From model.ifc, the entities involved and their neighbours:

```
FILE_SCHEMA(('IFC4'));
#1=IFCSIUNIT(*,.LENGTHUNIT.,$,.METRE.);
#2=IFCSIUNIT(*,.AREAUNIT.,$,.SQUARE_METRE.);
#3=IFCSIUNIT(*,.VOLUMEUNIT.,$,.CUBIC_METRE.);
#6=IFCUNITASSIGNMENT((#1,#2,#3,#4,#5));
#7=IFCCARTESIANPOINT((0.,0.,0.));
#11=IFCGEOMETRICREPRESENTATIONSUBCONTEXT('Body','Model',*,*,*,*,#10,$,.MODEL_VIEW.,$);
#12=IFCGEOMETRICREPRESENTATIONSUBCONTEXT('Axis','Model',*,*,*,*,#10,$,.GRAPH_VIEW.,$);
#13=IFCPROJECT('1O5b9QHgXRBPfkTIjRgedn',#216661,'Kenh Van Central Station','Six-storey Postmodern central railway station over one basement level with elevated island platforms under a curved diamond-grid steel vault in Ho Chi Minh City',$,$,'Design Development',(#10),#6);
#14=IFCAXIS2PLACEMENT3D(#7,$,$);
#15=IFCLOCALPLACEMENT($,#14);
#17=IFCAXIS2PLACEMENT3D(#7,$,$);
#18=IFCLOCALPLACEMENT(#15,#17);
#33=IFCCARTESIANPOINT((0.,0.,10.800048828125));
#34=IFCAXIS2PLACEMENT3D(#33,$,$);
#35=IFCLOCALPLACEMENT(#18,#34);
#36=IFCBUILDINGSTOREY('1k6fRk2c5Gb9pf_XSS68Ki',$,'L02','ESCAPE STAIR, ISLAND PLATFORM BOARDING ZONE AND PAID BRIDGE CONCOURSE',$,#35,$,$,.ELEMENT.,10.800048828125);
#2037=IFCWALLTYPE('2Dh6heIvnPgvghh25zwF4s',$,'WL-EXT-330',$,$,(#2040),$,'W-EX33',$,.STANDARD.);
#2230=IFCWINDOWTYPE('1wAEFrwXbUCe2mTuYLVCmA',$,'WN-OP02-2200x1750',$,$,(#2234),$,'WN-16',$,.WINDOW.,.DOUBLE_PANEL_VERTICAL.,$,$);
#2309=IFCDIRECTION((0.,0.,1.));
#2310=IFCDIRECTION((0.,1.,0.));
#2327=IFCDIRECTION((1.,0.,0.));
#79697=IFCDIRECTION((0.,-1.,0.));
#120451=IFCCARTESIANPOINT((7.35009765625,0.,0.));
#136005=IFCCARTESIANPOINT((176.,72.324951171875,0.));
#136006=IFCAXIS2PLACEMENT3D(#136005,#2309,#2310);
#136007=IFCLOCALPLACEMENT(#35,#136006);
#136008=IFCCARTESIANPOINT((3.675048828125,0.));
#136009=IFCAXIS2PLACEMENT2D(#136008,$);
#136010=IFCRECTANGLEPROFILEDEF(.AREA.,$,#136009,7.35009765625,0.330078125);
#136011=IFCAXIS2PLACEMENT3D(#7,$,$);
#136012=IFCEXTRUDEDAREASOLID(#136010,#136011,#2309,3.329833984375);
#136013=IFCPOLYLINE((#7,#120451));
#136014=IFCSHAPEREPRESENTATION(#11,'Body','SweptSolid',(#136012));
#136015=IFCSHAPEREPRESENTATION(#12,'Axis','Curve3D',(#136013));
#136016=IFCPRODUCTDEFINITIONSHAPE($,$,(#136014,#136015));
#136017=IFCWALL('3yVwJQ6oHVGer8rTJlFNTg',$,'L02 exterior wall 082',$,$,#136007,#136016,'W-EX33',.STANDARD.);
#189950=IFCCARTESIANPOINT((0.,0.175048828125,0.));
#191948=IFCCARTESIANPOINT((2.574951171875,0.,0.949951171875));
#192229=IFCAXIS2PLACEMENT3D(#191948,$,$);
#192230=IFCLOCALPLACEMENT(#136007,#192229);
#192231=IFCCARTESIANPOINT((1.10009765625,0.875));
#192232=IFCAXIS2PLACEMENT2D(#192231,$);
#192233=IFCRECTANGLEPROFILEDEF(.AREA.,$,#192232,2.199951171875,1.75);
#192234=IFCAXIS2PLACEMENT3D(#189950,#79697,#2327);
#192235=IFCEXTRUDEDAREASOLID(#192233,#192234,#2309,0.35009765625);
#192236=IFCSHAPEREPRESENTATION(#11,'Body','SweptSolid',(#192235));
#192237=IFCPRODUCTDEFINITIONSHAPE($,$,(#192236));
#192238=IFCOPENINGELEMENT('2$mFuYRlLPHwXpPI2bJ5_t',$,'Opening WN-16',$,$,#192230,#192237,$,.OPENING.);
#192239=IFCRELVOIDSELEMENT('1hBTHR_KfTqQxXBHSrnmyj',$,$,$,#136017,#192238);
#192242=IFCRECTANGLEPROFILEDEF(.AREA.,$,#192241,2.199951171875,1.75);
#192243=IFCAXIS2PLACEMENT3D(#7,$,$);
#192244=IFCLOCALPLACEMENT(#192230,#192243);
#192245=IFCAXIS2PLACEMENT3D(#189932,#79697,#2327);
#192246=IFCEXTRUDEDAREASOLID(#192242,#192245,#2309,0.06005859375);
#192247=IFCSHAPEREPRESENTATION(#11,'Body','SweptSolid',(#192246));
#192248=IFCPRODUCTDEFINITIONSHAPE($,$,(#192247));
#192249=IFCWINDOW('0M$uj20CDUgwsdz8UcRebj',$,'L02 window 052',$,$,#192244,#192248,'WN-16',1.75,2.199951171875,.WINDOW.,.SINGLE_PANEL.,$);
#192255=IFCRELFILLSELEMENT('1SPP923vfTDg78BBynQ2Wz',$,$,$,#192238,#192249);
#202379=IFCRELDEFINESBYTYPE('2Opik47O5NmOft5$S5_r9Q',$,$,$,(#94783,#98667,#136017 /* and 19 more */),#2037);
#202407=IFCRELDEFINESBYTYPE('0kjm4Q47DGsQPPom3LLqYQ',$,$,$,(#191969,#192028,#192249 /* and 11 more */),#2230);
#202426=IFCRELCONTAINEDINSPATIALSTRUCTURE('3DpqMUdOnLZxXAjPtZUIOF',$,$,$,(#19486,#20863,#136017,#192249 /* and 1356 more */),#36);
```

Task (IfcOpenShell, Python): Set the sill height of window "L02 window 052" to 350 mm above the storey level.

```python
import numpy as np
import ifcopenshell
import ifcopenshell.api.geometry
import ifcopenshell.geom
import ifcopenshell.util.element
import ifcopenshell.util.placement
import ifcopenshell.util.shape
import ifcopenshell.util.unit

model = ifcopenshell.open("model.ifc")
unit_scale = ifcopenshell.util.unit.calculate_unit_scale(model)

window = model.by_id(192249)
opening = window.FillsVoids[0].RelatingOpeningElement
storey = ifcopenshell.util.element.get_container(window, ifc_class="IfcBuildingStorey")
level = ifcopenshell.util.placement.get_local_placement(storey.ObjectPlacement)[2, 3]

# The opening's origin need not be at the sill, so measure its lowest point.
shape = ifcopenshell.geom.create_shape(ifcopenshell.geom.settings(), opening)
bottom = ifcopenshell.util.shape.get_shape_bottom_elevation(shape, shape.geometry) / unit_scale
dz = level + 0.35 - bottom

shift = np.array([0.0, 0.0, dz])
# The window is placed relative to its opening, so it follows when the opening moves.
matrix = ifcopenshell.util.placement.get_local_placement(opening.ObjectPlacement)
matrix[:3, 3] += shift
ifcopenshell.api.geometry.edit_object_placement(
    model, product=opening, matrix=matrix, is_si=False, should_transform_children=True
)

print(f"moved by {dz * unit_scale:+.3f} m")

model.write("model_v2.ifc")
```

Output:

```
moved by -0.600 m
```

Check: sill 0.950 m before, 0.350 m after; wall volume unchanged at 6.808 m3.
